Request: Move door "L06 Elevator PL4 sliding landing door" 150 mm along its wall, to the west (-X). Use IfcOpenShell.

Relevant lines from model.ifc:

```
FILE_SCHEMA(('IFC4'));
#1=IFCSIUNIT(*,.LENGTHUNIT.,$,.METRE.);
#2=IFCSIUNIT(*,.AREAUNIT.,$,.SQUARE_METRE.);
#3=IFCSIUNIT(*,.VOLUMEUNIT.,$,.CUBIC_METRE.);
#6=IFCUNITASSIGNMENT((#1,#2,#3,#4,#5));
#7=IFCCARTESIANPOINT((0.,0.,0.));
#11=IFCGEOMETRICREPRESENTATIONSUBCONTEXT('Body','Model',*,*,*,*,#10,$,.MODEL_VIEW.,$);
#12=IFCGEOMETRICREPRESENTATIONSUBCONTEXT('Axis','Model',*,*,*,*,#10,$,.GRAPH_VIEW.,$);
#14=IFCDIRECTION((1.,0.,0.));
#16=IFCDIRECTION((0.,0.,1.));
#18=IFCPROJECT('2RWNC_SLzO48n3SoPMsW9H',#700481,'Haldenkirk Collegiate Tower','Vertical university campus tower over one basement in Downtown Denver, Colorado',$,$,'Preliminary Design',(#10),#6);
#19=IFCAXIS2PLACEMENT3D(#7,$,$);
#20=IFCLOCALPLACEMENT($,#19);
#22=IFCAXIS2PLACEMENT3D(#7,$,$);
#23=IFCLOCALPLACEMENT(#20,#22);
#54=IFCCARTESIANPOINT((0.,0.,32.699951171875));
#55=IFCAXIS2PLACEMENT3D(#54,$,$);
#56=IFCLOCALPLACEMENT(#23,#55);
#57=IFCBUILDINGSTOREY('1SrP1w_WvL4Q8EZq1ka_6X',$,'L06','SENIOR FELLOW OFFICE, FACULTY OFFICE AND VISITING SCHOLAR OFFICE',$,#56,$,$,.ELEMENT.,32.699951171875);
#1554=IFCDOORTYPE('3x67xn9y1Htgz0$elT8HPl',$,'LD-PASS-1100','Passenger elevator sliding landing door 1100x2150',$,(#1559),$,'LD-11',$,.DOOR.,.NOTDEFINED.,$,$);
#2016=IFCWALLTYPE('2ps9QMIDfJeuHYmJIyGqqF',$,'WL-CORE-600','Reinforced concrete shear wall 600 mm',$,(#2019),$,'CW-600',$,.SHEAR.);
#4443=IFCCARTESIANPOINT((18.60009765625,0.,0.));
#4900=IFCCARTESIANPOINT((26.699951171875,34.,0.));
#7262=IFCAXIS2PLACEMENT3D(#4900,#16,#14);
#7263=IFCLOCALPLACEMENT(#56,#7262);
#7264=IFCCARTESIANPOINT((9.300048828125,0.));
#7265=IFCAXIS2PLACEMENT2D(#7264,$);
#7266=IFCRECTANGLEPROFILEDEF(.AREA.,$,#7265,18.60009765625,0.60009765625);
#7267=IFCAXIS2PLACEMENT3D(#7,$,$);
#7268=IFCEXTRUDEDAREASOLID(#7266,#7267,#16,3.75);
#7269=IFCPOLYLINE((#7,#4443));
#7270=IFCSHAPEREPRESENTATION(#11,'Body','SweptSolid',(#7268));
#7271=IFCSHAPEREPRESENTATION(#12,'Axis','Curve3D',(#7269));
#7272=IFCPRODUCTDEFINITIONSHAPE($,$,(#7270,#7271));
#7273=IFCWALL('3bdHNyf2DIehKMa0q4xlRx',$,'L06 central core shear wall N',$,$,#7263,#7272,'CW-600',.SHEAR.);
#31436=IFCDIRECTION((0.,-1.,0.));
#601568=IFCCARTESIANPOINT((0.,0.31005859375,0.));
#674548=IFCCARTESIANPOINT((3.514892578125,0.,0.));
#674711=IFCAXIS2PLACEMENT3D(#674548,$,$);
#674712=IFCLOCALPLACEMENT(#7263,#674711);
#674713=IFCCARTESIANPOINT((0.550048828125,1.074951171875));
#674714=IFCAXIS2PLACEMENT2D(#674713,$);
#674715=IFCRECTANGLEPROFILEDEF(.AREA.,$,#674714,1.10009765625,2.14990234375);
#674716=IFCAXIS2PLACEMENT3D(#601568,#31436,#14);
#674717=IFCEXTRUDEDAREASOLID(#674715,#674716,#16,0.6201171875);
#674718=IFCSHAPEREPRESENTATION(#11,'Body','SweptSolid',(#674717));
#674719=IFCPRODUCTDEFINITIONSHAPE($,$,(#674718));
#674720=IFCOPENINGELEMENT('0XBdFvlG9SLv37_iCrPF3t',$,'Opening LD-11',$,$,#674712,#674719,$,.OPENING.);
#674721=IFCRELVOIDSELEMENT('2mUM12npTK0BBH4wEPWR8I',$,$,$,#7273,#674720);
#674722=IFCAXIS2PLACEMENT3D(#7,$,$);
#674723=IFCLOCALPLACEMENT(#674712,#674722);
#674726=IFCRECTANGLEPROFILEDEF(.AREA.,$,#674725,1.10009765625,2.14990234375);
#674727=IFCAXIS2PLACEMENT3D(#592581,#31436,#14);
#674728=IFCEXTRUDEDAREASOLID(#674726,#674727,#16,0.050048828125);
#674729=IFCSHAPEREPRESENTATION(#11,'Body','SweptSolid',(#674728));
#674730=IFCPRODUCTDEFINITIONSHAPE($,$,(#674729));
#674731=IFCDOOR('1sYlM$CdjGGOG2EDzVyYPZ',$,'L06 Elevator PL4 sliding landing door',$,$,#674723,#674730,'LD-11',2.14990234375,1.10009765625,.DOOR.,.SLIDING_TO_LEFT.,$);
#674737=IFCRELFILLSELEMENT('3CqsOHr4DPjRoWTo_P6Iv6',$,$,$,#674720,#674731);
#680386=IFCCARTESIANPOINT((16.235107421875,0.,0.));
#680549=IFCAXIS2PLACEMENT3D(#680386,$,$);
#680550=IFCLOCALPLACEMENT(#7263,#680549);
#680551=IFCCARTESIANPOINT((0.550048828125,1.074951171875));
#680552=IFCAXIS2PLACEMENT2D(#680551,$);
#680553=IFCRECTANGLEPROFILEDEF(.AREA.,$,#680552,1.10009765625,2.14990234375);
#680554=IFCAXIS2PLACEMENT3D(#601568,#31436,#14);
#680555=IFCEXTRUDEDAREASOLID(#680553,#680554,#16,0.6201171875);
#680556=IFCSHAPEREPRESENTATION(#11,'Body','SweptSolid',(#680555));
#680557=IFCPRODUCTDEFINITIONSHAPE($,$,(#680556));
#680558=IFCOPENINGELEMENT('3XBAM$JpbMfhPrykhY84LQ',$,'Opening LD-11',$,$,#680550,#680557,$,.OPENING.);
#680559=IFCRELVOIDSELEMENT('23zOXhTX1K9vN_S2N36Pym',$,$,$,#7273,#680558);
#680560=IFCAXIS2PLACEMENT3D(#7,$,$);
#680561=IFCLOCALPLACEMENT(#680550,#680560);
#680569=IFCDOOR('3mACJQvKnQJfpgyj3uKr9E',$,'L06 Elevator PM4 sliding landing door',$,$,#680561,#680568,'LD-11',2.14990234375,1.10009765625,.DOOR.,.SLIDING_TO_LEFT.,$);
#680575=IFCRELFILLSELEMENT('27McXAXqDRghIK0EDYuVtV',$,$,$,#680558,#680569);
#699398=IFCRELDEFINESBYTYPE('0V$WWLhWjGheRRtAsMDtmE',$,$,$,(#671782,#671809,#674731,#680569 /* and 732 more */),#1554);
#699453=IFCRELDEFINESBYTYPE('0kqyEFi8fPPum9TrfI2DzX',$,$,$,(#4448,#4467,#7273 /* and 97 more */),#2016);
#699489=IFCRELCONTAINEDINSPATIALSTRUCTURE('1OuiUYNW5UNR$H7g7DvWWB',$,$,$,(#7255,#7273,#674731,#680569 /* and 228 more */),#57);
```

```python
import ifcopenshell
import ifcopenshell.api.geometry
import ifcopenshell.util.placement
import ifcopenshell.util.unit

model = ifcopenshell.open("model.ifc")
unit_scale = ifcopenshell.util.unit.calculate_unit_scale(model)

door = model.by_id(674731)
opening = door.FillsVoids[0].RelatingOpeningElement
wall = opening.VoidsElements[0].RelatingBuildingElement

wall_matrix = ifcopenshell.util.placement.get_local_placement(wall.ObjectPlacement)
shift = wall_matrix[:3, 0] * -0.15 / unit_scale
before = ifcopenshell.util.placement.get_local_placement(door.ObjectPlacement)[:3, 3].copy()

# The door is placed relative to its opening, so it follows when the opening moves.
matrix = ifcopenshell.util.placement.get_local_placement(opening.ObjectPlacement)
matrix[:3, 3] += shift
ifcopenshell.api.geometry.edit_object_placement(
    model, product=opening, matrix=matrix, is_si=False, should_transform_children=True
)

after = ifcopenshell.util.placement.get_local_placement(door.ObjectPlacement)[:3, 3]
print("door moved by", (after - before).round(3) + 0.0)

model.write("model_edited.ifc")
```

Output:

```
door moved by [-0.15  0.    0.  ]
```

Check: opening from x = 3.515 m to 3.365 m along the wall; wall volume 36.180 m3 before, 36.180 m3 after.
